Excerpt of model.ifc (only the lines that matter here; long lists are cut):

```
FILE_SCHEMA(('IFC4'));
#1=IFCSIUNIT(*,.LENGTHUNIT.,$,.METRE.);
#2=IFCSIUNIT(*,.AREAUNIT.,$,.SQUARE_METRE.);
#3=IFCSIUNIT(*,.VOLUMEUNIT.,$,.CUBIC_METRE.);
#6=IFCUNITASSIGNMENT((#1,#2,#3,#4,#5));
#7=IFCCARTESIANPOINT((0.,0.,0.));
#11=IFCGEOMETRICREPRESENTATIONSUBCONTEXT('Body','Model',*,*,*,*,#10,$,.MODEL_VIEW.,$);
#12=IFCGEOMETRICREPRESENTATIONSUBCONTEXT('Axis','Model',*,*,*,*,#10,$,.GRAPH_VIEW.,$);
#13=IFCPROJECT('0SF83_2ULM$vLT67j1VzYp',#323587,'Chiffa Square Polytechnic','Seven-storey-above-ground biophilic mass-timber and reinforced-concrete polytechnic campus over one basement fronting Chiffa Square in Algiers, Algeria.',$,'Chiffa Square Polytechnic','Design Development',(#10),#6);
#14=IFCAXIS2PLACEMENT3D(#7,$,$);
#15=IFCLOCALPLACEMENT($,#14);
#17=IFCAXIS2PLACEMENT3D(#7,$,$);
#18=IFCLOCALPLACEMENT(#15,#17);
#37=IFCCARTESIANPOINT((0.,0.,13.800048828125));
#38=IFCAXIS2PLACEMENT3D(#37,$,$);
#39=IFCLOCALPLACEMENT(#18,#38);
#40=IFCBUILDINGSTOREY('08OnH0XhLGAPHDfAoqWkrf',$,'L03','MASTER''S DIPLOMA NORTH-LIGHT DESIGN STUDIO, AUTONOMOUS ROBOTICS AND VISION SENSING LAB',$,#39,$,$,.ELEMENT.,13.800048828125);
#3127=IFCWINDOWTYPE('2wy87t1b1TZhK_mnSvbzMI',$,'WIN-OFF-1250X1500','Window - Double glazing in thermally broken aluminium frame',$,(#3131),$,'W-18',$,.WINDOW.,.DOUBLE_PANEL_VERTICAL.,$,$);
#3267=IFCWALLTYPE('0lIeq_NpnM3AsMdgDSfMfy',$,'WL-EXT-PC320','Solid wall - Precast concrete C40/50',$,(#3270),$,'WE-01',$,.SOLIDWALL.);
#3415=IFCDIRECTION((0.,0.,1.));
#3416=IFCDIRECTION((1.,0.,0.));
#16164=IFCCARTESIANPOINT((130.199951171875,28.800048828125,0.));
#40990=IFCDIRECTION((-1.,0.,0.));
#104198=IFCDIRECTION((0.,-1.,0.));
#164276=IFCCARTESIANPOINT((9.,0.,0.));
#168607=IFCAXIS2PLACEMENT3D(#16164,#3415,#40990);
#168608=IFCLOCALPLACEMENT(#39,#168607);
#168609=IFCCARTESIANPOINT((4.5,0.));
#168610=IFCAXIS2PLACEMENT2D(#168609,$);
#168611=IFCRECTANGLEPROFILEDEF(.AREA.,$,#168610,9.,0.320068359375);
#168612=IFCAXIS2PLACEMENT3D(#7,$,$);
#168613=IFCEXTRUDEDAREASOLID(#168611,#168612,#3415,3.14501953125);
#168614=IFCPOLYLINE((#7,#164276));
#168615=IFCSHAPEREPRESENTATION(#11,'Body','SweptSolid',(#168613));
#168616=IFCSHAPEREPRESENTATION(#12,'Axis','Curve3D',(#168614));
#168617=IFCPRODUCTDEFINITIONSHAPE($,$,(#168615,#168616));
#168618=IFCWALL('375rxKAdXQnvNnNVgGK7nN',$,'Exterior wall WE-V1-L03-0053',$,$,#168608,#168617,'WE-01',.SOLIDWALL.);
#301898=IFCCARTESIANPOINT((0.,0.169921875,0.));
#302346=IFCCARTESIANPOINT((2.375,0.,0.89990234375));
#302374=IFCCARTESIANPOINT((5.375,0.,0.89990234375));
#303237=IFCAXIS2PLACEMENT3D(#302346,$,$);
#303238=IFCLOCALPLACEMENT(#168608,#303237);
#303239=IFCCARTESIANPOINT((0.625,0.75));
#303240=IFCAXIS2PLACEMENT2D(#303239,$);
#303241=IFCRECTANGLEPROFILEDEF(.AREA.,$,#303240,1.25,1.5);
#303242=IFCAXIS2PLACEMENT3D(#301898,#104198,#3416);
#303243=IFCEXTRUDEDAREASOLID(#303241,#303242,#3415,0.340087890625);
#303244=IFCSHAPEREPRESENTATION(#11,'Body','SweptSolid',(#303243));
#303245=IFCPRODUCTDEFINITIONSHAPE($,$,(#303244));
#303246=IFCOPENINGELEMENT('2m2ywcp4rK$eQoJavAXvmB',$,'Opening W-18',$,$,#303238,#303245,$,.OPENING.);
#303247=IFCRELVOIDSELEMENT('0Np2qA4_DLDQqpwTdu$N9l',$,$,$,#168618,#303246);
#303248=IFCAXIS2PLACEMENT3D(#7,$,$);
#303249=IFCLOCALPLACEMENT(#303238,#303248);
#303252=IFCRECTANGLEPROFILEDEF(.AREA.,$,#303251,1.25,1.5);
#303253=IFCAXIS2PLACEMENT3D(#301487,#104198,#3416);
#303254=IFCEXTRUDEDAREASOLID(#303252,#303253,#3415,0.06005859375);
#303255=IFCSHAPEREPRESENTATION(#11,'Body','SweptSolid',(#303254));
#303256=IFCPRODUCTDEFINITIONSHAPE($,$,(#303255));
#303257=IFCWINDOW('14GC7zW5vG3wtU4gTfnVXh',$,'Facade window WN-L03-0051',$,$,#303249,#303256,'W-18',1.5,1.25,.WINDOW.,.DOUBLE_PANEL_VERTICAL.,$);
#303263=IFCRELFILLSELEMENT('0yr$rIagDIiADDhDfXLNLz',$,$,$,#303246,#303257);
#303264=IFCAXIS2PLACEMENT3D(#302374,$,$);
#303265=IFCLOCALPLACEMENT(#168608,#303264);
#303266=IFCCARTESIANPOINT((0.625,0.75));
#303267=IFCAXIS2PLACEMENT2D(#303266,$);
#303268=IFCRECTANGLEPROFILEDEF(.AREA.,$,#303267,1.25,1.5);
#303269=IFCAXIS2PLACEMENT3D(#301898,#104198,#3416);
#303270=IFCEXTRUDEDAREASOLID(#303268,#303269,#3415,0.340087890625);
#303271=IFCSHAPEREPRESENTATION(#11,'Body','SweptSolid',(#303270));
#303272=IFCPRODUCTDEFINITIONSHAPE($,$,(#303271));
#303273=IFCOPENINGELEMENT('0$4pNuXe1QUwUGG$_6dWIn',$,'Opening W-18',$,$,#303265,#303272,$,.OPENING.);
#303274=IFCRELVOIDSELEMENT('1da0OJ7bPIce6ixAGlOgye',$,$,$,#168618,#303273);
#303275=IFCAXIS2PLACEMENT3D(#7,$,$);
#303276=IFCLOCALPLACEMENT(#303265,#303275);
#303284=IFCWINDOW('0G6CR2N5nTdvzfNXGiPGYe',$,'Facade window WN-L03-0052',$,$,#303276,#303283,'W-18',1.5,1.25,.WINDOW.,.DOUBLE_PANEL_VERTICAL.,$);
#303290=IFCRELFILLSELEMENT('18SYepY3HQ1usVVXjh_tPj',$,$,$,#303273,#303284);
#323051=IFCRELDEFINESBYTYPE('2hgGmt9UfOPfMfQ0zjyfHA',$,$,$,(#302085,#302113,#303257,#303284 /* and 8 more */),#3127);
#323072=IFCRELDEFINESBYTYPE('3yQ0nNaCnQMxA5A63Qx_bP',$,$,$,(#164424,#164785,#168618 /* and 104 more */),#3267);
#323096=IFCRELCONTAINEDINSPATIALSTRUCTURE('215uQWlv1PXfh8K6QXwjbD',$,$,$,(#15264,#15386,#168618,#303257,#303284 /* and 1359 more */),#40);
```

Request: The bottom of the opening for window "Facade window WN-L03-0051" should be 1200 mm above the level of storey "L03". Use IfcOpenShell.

```python
import numpy as np
import ifcopenshell
import ifcopenshell.api.geometry
import ifcopenshell.geom
import ifcopenshell.util.element
import ifcopenshell.util.placement
import ifcopenshell.util.shape
import ifcopenshell.util.unit

model = ifcopenshell.open("model.ifc")
unit_scale = ifcopenshell.util.unit.calculate_unit_scale(model)

window = model.by_guid("14GC7zW5vG3wtU4gTfnVXh")
opening = window.FillsVoids[0].RelatingOpeningElement
storey = ifcopenshell.util.element.get_container(window, ifc_class="IfcBuildingStorey")
level = ifcopenshell.util.placement.get_local_placement(storey.ObjectPlacement)[2, 3]

# The opening's origin need not be at the sill, so measure its lowest point.
shape = ifcopenshell.geom.create_shape(ifcopenshell.geom.settings(), opening)
bottom = ifcopenshell.util.shape.get_shape_bottom_elevation(shape, shape.geometry) / unit_scale
dz = level + 1.2 / unit_scale - bottom

shift = np.array([0.0, 0.0, dz])
# The window is placed relative to its opening, so it follows when the opening moves.
matrix = ifcopenshell.util.placement.get_local_placement(opening.ObjectPlacement)
matrix[:3, 3] += shift
ifcopenshell.api.geometry.edit_object_placement(
    model, product=opening, matrix=matrix, is_si=False, should_transform_children=True
)

print(f"moved by {dz * unit_scale:+.3f} m")

model.write("model_updated.ifc")
```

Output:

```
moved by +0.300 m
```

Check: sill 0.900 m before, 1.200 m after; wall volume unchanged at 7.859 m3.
